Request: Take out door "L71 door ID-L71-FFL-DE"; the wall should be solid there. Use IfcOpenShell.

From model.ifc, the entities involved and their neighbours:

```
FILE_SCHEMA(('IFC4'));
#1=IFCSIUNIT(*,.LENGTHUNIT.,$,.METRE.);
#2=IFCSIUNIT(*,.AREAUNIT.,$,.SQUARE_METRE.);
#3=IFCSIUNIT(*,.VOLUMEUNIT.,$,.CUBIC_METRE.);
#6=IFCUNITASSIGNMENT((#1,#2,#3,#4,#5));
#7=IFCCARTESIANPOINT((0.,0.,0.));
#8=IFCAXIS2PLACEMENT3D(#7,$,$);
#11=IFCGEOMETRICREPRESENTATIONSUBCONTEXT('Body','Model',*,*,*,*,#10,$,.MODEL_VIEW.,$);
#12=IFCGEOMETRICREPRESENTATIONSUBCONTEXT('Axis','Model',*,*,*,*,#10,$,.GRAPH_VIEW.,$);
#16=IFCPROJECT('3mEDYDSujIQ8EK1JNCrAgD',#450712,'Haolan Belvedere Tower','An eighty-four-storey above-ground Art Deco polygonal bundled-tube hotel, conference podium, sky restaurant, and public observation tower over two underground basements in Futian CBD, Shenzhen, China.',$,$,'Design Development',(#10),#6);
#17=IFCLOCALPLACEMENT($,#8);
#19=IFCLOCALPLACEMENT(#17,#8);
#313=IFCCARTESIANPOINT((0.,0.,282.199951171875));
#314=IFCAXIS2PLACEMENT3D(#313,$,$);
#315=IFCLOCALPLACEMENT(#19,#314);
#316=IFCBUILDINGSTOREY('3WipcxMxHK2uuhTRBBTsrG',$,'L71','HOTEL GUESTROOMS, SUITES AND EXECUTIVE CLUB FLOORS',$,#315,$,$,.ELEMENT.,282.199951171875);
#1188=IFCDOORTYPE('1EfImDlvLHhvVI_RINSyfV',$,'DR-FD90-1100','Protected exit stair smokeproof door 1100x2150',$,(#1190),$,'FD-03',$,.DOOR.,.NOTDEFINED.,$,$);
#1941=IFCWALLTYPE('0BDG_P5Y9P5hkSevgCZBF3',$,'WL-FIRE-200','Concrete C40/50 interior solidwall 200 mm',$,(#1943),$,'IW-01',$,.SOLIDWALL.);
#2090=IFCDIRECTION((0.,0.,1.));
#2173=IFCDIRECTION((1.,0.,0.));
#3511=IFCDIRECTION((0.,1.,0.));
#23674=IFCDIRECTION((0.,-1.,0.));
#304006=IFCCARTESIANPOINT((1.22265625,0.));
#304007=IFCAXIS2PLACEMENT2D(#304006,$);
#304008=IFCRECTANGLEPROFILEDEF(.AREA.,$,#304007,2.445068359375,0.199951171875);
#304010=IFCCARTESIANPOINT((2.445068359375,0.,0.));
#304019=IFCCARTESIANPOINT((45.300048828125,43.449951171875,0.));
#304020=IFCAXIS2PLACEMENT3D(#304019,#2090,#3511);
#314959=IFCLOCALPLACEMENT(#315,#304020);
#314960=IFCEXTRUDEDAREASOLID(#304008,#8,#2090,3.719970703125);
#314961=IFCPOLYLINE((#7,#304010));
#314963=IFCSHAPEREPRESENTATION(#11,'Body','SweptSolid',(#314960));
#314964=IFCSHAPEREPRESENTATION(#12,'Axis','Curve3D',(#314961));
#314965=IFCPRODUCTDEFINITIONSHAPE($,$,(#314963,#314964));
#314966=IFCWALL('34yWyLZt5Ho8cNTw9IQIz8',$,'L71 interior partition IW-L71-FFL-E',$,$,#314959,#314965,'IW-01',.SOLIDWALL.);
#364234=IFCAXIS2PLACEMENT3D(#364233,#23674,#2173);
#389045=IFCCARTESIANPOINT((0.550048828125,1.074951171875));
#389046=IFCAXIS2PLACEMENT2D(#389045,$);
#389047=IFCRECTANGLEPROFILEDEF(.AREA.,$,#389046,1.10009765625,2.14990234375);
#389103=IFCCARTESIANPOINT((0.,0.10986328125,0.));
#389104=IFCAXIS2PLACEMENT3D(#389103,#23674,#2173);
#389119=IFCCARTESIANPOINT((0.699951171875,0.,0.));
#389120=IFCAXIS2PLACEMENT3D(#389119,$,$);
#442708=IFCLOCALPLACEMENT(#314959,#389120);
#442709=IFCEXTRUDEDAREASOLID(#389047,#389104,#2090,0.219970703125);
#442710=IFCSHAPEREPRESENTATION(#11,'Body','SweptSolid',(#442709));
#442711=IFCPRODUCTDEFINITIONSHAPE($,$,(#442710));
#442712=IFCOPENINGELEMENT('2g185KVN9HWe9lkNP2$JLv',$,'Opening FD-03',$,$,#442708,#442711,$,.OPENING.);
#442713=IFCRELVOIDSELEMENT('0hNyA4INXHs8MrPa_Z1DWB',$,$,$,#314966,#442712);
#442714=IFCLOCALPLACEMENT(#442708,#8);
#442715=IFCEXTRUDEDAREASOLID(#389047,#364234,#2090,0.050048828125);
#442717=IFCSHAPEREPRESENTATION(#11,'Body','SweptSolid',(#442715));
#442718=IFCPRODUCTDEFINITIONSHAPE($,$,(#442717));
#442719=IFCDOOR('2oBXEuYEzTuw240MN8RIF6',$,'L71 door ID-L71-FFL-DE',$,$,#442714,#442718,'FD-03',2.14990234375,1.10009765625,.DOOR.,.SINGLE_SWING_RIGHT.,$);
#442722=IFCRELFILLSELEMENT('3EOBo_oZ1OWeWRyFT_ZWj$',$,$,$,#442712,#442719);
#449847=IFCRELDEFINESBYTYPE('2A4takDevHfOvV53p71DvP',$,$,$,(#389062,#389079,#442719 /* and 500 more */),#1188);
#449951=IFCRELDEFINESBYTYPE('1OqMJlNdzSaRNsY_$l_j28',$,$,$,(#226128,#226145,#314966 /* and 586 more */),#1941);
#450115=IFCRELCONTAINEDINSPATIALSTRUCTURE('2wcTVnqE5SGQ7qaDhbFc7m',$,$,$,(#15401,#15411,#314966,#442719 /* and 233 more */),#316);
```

```python
import ifcopenshell
import ifcopenshell.api.feature
import ifcopenshell.api.root
import ifcopenshell.geom
import ifcopenshell.util.shape

model = ifcopenshell.open("model.ifc")
settings = ifcopenshell.geom.settings()


def volume(element):
    """Net volume in cubic metres, openings subtracted."""
    shape = ifcopenshell.geom.create_shape(settings, element)
    return ifcopenshell.util.shape.get_volume(shape.geometry)


door = model.by_guid("2oBXEuYEzTuw240MN8RIF6")
opening = door.FillsVoids[0].RelatingOpeningElement
wall = opening.VoidsElements[0].RelatingBuildingElement
before = volume(wall)

ifcopenshell.api.root.remove_product(model, product=door)
ifcopenshell.api.feature.remove_feature(model, feature=opening)

after = volume(wall)

print(f"wall volume {before:.3f} -> {after:.3f} m3")

model.write("model_updated.ifc")
```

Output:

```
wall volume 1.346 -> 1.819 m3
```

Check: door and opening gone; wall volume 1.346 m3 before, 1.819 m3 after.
